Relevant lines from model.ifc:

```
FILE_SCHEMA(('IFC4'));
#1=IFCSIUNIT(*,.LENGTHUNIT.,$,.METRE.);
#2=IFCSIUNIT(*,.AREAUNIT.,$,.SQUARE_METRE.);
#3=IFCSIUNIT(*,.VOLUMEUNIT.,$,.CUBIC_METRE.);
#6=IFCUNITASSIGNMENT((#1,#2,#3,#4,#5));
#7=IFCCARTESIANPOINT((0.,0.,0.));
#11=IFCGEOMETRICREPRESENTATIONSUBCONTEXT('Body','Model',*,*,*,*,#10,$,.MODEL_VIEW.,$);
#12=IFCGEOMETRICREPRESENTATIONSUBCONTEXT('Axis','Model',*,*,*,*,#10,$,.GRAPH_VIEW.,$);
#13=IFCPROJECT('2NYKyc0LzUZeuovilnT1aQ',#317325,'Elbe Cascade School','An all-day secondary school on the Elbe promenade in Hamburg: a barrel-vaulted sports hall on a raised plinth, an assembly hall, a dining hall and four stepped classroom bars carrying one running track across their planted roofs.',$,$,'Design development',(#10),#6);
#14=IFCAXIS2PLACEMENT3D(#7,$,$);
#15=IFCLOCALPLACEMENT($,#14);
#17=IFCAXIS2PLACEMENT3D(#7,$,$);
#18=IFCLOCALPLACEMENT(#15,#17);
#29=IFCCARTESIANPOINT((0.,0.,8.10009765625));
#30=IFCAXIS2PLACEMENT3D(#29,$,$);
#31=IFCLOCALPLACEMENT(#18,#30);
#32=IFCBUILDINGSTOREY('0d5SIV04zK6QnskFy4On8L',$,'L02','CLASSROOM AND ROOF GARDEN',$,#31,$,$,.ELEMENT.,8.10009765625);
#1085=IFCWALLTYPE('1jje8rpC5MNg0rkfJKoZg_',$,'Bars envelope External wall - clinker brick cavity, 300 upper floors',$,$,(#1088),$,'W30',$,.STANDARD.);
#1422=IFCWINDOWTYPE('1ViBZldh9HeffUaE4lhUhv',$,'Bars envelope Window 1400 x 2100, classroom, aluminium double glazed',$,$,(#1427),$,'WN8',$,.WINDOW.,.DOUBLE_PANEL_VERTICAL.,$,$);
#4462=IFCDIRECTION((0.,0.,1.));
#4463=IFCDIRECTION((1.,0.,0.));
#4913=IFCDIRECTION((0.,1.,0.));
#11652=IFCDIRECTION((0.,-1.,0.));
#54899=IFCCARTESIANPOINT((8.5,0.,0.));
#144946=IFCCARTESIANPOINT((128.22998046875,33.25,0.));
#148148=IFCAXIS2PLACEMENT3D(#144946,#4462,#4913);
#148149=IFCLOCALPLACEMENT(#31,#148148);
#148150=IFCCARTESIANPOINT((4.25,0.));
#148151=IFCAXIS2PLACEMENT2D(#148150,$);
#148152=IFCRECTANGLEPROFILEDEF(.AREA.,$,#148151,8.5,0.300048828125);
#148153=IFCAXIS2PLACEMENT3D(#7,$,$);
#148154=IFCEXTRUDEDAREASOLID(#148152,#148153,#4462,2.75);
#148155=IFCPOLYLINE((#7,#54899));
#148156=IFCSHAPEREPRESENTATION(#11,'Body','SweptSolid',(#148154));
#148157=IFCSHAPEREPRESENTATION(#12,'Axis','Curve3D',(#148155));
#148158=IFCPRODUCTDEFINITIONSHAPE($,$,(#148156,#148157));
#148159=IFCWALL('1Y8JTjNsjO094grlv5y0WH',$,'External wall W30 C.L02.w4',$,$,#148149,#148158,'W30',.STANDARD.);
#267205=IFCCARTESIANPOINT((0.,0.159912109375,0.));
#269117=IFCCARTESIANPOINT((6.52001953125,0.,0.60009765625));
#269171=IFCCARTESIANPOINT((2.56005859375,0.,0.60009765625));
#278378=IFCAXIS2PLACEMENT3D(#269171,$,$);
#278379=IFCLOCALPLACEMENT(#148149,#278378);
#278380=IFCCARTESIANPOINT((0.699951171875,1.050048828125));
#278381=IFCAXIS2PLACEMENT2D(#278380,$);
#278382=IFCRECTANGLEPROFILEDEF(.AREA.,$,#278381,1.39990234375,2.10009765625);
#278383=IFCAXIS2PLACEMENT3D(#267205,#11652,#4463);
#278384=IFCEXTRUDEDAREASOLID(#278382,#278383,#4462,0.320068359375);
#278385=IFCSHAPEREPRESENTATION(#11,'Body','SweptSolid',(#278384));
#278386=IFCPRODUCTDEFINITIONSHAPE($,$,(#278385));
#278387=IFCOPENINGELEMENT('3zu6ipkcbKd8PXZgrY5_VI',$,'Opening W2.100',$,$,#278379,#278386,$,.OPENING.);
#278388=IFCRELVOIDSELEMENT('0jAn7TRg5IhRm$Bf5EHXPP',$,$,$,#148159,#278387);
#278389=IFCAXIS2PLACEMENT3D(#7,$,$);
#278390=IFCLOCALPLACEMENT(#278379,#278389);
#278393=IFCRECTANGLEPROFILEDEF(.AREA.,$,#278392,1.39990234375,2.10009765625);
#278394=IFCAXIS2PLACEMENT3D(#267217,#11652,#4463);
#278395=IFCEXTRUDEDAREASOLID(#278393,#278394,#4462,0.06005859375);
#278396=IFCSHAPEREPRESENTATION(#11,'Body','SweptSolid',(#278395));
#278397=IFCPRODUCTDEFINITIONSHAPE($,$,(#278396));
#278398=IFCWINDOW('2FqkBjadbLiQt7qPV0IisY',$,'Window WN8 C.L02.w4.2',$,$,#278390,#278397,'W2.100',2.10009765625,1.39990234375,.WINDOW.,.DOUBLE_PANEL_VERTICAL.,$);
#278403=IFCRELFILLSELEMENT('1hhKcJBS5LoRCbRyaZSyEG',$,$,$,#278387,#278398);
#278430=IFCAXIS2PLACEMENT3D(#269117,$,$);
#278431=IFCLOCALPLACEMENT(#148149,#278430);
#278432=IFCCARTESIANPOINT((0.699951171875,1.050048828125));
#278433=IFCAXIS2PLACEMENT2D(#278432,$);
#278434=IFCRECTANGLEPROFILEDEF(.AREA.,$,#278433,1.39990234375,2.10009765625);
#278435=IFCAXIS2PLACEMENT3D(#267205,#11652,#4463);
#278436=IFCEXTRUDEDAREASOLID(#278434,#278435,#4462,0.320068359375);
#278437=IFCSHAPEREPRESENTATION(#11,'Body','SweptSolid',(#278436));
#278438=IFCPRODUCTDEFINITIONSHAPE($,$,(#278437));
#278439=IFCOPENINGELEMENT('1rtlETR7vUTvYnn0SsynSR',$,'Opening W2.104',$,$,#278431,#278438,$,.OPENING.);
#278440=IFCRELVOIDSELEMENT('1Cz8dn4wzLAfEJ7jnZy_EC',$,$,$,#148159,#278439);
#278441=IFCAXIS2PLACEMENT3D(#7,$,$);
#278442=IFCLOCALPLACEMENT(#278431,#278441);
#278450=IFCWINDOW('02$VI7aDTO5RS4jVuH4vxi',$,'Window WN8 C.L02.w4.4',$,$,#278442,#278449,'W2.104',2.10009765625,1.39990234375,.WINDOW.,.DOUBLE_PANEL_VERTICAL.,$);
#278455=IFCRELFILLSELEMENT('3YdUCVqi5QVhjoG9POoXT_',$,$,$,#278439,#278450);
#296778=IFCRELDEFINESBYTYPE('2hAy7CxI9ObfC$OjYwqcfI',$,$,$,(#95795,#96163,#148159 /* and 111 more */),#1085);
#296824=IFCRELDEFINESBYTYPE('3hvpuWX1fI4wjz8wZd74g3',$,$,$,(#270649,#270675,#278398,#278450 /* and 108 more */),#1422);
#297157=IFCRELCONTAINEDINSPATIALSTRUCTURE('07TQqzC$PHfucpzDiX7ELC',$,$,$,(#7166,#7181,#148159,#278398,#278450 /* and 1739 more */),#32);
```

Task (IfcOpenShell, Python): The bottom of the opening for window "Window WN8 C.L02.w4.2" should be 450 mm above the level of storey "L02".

```python
import numpy as np
import ifcopenshell
import ifcopenshell.api.geometry
import ifcopenshell.geom
import ifcopenshell.util.element
import ifcopenshell.util.placement
import ifcopenshell.util.shape
import ifcopenshell.util.unit

model = ifcopenshell.open("model.ifc")
unit_scale = ifcopenshell.util.unit.calculate_unit_scale(model)

window = model.by_guid("2FqkBjadbLiQt7qPV0IisY")
opening = window.FillsVoids[0].RelatingOpeningElement
storey = ifcopenshell.util.element.get_container(window, ifc_class="IfcBuildingStorey")
level = ifcopenshell.util.placement.get_local_placement(storey.ObjectPlacement)[2, 3]

# The opening's origin need not be at the sill, so measure its lowest point.
shape = ifcopenshell.geom.create_shape(ifcopenshell.geom.settings(), opening)
bottom = ifcopenshell.util.shape.get_shape_bottom_elevation(shape, shape.geometry) / unit_scale
dz = level + 0.45 / unit_scale - bottom

shift = np.array([0.0, 0.0, dz])
# The window is placed relative to its opening, so it follows when the opening moves.
matrix = ifcopenshell.util.placement.get_local_placement(opening.ObjectPlacement)
matrix[:3, 3] += shift
ifcopenshell.api.geometry.edit_object_placement(
    model, product=opening, matrix=matrix, is_si=False, should_transform_children=True
)

print(f"moved by {dz * unit_scale:+.3f} m")

model.write("model_edited.ifc")
```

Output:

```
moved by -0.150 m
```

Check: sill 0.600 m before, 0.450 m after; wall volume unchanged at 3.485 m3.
